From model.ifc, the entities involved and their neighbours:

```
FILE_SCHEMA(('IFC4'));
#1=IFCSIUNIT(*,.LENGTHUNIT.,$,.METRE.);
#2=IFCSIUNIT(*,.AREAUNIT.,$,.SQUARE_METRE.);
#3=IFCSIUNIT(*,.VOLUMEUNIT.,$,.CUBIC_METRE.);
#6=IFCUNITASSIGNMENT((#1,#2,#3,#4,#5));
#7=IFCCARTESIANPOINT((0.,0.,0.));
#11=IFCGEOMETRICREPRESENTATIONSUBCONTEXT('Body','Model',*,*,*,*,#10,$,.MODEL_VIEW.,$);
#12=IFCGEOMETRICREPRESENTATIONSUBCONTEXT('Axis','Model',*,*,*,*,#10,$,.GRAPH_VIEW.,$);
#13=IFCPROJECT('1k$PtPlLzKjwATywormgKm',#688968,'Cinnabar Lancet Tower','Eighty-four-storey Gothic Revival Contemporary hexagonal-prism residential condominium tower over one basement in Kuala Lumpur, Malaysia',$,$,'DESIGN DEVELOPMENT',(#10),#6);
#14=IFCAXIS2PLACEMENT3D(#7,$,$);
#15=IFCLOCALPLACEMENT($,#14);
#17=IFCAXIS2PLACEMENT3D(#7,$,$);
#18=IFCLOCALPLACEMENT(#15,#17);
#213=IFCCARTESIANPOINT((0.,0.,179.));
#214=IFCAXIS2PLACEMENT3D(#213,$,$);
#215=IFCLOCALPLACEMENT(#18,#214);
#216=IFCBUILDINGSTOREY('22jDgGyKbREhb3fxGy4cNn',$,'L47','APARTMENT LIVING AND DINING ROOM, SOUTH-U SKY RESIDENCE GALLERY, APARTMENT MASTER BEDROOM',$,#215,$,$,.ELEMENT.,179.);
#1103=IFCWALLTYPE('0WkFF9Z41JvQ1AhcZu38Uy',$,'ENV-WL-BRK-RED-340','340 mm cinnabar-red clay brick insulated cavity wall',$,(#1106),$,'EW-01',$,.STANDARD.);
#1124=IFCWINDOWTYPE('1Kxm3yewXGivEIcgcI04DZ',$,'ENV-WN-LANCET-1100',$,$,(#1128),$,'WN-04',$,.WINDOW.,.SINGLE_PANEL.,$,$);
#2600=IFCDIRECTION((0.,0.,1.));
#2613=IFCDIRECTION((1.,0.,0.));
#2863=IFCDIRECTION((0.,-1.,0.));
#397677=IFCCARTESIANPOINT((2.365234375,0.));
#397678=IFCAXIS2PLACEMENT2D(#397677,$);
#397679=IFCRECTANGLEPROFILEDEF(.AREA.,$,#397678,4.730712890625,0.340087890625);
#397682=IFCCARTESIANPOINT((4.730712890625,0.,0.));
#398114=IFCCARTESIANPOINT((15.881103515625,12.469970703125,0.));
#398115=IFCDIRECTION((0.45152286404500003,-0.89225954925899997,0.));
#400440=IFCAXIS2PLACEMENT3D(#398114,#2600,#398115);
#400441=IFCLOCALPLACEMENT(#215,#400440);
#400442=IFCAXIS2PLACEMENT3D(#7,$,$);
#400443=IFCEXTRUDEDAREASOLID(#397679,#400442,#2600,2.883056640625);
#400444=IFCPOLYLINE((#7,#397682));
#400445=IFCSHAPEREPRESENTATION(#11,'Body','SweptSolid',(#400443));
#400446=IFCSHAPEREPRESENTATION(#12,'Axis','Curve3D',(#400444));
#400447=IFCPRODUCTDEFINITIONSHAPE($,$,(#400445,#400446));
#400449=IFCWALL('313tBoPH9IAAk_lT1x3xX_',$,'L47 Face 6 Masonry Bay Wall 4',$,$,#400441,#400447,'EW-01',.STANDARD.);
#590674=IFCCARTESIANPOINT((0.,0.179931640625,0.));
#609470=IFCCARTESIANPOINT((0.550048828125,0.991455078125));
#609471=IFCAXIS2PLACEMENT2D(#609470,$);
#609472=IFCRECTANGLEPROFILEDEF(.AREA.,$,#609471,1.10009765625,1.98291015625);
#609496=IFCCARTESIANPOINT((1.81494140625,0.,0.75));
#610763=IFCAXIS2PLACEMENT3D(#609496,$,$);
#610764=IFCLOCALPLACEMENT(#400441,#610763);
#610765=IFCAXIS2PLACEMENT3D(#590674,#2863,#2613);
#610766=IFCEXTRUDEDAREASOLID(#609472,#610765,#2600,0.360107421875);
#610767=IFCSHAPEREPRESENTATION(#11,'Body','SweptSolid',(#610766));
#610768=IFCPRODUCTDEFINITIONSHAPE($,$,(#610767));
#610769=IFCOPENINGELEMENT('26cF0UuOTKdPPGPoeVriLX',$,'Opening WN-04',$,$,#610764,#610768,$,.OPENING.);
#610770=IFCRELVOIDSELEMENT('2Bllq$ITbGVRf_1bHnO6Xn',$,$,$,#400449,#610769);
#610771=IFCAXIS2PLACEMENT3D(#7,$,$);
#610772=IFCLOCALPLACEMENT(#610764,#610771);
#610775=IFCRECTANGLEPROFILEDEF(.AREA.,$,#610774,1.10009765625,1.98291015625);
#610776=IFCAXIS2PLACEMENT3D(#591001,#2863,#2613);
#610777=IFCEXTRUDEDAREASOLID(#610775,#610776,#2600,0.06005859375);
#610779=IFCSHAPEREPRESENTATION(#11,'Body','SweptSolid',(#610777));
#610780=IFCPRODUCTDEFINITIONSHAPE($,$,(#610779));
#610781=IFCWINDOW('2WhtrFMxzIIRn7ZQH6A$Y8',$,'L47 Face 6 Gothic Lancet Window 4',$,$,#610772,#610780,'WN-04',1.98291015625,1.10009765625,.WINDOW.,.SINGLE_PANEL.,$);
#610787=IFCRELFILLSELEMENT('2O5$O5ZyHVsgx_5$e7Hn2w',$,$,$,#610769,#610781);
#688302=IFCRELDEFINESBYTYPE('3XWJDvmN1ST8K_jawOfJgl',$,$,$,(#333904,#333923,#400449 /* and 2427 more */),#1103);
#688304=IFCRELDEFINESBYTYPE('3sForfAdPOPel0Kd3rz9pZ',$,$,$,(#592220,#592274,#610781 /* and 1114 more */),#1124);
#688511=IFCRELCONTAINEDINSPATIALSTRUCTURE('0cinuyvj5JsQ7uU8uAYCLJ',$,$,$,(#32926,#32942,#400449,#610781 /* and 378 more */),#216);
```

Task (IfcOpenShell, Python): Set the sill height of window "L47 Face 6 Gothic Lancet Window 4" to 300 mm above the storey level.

```python
import numpy as np
import ifcopenshell
import ifcopenshell.api.geometry
import ifcopenshell.geom
import ifcopenshell.util.element
import ifcopenshell.util.placement
import ifcopenshell.util.shape
import ifcopenshell.util.unit

model = ifcopenshell.open("model.ifc")
unit_scale = ifcopenshell.util.unit.calculate_unit_scale(model)

window = model.by_id(610781)
opening = window.FillsVoids[0].RelatingOpeningElement
storey = ifcopenshell.util.element.get_container(window, ifc_class="IfcBuildingStorey")
level = ifcopenshell.util.placement.get_local_placement(storey.ObjectPlacement)[2, 3]

# The opening's origin need not be at the sill, so measure its lowest point.
shape = ifcopenshell.geom.create_shape(ifcopenshell.geom.settings(), opening)
bottom = ifcopenshell.util.shape.get_shape_bottom_elevation(shape, shape.geometry) / unit_scale
dz = level + 0.3 / unit_scale - bottom

shift = np.array([0.0, 0.0, dz])
# The window is placed relative to its opening, so it follows when the opening moves.
matrix = ifcopenshell.util.placement.get_local_placement(opening.ObjectPlacement)
matrix[:3, 3] += shift
ifcopenshell.api.geometry.edit_object_placement(
    model, product=opening, matrix=matrix, is_si=False, should_transform_children=True
)

print(f"moved by {dz * unit_scale:+.3f} m")

model.write("model-out.ifc")
```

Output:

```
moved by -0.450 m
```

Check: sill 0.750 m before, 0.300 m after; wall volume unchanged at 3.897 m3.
